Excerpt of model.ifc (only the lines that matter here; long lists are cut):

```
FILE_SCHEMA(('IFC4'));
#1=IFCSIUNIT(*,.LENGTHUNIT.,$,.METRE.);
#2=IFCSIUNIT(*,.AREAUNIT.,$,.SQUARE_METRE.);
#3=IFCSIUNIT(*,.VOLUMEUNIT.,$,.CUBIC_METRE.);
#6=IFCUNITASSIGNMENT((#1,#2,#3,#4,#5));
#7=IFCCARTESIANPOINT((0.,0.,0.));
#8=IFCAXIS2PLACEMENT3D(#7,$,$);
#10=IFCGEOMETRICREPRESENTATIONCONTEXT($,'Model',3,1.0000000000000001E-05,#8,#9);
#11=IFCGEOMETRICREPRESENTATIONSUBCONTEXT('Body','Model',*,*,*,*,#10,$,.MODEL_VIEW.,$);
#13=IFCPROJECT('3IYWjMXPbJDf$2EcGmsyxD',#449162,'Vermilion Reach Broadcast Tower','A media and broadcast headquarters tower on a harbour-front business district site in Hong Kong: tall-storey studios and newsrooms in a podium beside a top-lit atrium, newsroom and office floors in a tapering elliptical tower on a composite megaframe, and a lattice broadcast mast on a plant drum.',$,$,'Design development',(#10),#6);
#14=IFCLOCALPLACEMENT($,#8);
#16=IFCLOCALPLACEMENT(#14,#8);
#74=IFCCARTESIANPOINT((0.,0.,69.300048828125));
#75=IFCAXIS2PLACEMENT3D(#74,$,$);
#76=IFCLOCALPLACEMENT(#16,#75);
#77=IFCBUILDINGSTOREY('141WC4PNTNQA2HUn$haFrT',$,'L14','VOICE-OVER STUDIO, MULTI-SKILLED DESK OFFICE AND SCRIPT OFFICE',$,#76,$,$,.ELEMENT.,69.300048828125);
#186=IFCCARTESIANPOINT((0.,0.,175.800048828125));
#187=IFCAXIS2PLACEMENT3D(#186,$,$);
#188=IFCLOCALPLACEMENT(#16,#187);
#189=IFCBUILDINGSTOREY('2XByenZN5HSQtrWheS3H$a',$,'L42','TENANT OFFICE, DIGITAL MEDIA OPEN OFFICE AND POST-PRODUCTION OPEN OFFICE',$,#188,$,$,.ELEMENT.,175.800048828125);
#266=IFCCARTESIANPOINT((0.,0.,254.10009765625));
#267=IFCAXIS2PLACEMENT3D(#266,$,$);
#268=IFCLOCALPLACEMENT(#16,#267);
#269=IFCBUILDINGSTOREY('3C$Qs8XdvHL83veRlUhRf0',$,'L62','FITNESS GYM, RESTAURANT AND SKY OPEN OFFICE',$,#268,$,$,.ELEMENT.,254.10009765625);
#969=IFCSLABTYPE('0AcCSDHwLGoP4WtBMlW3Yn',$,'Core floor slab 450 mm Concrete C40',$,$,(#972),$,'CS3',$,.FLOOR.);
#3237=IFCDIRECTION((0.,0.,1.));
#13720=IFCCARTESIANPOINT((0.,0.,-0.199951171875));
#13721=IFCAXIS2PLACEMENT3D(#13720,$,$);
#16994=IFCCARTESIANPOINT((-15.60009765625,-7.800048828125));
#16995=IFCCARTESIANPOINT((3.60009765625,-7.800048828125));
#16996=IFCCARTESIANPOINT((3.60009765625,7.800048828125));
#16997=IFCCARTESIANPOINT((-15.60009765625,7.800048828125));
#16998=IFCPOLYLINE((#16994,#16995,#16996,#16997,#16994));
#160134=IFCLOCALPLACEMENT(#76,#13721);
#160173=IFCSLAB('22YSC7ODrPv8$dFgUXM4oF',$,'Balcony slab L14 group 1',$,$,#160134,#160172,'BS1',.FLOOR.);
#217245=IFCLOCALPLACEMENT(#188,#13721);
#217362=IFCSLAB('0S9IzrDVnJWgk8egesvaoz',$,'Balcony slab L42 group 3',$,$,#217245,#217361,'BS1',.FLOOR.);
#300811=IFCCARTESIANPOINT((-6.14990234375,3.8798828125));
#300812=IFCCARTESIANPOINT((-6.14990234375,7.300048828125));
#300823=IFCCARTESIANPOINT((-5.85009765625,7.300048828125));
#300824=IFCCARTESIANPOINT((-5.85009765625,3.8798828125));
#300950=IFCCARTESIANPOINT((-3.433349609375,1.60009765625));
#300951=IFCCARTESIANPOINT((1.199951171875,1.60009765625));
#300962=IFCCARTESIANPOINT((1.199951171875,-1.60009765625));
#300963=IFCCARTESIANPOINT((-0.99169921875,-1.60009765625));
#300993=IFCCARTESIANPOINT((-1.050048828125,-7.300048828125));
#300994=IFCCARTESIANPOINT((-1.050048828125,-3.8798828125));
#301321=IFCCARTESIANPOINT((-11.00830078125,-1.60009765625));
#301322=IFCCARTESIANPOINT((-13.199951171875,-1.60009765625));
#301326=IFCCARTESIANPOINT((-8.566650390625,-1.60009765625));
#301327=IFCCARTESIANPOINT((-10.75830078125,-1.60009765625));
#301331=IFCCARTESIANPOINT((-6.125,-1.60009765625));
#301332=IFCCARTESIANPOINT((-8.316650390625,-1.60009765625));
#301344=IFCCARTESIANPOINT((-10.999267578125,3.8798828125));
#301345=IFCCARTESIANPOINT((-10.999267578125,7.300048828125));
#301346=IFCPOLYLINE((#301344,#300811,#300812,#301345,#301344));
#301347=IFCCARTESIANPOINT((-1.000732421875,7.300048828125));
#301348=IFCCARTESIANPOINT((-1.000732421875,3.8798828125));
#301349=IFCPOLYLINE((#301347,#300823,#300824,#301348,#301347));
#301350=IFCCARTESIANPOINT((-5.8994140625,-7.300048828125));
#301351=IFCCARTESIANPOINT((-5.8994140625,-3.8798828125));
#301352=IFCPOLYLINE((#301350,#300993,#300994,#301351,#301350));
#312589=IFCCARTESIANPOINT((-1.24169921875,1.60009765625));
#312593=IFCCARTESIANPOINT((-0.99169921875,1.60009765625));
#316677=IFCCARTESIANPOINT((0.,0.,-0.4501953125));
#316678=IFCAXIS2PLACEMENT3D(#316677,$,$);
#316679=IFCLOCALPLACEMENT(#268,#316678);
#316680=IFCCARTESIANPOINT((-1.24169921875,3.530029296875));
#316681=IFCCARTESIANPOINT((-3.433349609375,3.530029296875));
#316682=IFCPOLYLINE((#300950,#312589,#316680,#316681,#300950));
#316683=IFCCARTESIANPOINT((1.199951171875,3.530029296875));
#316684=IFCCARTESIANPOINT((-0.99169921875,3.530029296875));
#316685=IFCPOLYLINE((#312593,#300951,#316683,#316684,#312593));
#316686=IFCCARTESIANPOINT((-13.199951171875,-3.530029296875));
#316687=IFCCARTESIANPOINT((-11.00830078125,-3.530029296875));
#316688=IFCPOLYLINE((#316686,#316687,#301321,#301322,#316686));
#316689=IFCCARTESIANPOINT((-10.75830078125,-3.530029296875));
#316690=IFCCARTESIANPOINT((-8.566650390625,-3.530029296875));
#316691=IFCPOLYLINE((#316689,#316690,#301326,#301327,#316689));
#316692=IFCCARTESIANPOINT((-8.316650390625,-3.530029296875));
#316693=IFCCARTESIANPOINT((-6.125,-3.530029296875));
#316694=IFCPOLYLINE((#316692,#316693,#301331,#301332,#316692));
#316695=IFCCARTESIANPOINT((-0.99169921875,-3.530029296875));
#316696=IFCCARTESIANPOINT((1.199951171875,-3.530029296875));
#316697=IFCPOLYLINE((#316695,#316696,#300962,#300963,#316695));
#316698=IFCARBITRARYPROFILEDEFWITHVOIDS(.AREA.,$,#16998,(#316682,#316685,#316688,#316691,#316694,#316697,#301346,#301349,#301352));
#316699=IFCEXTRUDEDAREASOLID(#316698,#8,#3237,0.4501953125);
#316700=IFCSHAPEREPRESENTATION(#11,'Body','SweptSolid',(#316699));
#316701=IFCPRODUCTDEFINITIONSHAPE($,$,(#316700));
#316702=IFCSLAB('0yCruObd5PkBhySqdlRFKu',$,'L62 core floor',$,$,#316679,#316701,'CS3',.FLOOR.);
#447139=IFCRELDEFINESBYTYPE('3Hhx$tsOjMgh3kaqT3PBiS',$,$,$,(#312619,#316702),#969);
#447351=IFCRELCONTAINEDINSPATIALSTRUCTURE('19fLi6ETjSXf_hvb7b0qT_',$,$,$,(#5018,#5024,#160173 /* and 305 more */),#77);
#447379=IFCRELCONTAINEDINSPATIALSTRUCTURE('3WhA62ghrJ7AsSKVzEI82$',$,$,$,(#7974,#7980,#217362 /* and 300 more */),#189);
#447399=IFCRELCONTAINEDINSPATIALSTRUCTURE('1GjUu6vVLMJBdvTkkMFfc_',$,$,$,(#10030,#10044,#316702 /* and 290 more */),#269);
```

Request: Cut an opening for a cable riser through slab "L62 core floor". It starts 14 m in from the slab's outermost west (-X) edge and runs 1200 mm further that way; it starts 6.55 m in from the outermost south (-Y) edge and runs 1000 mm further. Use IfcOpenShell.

```python
import numpy as np
import ifcopenshell
import ifcopenshell.api.feature
import ifcopenshell.api.geometry
import ifcopenshell.api.root
import ifcopenshell.geom
import ifcopenshell.util.placement
import ifcopenshell.util.representation
import ifcopenshell.util.shape
import ifcopenshell.util.unit

model = ifcopenshell.open("model.ifc")
unit_scale = ifcopenshell.util.unit.calculate_unit_scale(model)
settings = ifcopenshell.geom.settings()


def volume(element):
    """Net volume in cubic metres, openings subtracted."""
    shape = ifcopenshell.geom.create_shape(settings, element)
    return ifcopenshell.util.shape.get_volume(shape.geometry)


slab = model.by_guid("0yCruObd5PkBhySqdlRFKu")
before = volume(slab)

# Extent in the slab's own axes, in metres. The edges named are its -X and -Y sides.
slab_shape = ifcopenshell.geom.create_shape(settings, slab)
vertices = ifcopenshell.util.shape.get_vertices(slab_shape.geometry)
x_min, y_min, bottom = vertices.min(axis=0)
top = vertices[:, 2].max()

opening = ifcopenshell.api.root.create_entity(model, ifc_class="IfcOpeningElement", name="Cable riser opening", predefined_type="OPENING")
context = ifcopenshell.util.representation.get_context(model, "Model", "Body", "MODEL_VIEW")
width, depth = 1.2, 1
outline = [(0.0, 0.0), (width, 0.0), (width, depth), (0.0, depth), (0.0, 0.0)]
# Overshoot both faces by 50 mm so the cut is clean.
shape = ifcopenshell.api.geometry.add_slab_representation(
    model, context=context, depth=top - bottom + 0.1, polyline=outline
)
ifcopenshell.api.geometry.assign_representation(model, product=opening, representation=shape)

matrix = ifcopenshell.util.placement.get_local_placement(slab.ObjectPlacement)
matrix[:, 3] = matrix @ np.append(np.array([x_min + 14, y_min + 6.55, bottom - 0.05]) / unit_scale, 1.0)
ifcopenshell.api.geometry.edit_object_placement(model, product=opening, matrix=matrix, is_si=False)
ifcopenshell.api.feature.add_feature(model, feature=opening, element=slab)

after = volume(slab)

print(f"slab volume {before:.3f} -> {after:.3f} m3")

model.write("model_v2.ifc")
```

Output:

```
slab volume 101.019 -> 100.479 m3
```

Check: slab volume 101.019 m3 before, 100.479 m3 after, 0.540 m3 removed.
